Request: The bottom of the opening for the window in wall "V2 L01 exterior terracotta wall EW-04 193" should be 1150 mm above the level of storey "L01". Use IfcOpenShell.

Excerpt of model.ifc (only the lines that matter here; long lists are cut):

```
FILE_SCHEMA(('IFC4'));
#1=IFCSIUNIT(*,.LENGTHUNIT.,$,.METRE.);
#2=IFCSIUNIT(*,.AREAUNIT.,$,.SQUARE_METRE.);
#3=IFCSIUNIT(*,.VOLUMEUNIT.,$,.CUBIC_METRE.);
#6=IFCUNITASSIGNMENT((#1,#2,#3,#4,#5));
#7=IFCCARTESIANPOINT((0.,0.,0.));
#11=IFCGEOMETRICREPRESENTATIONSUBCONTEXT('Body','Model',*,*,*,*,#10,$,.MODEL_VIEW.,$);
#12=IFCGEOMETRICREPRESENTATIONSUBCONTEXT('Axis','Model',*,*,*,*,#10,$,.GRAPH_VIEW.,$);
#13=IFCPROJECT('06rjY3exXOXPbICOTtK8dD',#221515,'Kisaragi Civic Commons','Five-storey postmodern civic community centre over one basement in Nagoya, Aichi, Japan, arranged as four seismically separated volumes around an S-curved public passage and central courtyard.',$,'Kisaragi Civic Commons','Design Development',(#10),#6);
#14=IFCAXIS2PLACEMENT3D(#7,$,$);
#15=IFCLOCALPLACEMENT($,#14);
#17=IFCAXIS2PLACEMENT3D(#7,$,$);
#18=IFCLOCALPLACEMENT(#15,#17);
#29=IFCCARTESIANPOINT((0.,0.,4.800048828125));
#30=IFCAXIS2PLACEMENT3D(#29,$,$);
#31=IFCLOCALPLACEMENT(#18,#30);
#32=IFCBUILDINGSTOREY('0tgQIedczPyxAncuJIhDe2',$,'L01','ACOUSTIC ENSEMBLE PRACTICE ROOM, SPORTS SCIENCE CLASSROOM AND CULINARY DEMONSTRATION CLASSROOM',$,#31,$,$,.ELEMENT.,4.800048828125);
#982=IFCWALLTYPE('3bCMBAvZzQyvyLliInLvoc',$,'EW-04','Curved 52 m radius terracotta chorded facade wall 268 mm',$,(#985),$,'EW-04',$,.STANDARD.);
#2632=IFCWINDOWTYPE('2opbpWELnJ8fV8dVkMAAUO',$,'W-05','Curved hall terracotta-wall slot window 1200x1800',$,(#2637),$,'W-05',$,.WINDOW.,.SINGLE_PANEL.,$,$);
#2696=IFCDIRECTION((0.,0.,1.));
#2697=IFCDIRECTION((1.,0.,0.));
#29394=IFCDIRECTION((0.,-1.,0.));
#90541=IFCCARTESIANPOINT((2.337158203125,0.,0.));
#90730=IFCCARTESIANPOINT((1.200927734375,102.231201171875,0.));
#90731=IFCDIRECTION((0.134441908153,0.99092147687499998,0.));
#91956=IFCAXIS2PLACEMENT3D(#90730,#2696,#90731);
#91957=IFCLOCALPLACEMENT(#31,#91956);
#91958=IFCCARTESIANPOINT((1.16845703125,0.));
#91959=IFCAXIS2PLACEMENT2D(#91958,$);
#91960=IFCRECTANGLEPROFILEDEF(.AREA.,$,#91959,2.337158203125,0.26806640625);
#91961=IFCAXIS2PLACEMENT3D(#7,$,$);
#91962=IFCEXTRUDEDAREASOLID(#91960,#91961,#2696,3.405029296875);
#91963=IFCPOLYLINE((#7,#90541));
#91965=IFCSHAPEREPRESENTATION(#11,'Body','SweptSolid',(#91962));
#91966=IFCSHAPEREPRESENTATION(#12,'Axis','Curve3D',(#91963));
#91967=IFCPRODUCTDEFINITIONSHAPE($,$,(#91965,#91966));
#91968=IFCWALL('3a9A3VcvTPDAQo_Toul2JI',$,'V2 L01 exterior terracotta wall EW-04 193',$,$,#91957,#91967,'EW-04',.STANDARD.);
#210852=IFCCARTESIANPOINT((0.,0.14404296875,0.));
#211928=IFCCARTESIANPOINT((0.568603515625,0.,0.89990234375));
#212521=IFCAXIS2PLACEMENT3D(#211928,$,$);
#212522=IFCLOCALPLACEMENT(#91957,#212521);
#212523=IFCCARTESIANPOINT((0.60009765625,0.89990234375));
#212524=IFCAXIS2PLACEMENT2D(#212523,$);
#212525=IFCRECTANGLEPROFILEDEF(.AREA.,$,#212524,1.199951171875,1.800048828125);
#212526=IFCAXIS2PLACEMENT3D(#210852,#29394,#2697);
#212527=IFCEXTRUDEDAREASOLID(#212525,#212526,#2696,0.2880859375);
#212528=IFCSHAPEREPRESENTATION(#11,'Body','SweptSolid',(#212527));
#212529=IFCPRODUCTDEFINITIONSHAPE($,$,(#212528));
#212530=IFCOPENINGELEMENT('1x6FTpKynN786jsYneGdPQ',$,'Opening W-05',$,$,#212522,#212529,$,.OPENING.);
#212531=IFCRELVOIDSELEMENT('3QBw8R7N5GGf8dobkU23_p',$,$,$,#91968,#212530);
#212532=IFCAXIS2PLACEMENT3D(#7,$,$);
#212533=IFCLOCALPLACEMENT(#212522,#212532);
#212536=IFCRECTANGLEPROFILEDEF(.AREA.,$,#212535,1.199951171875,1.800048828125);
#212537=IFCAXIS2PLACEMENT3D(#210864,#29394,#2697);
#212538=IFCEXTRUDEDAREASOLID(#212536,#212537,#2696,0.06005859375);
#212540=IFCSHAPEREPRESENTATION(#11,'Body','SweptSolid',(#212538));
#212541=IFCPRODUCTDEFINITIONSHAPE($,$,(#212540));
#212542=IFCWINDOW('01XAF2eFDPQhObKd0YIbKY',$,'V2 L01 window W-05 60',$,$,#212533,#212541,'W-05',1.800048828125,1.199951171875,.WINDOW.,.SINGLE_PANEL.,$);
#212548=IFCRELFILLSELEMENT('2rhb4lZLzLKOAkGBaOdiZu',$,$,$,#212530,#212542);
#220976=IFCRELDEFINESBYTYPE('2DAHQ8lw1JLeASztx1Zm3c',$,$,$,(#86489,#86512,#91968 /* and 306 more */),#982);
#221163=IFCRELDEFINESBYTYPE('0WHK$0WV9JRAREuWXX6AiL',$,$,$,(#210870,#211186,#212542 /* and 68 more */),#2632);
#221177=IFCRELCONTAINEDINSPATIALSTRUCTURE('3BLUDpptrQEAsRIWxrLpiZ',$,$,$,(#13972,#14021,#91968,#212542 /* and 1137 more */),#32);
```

```python
import numpy as np
import ifcopenshell
import ifcopenshell.api.geometry
import ifcopenshell.geom
import ifcopenshell.util.element
import ifcopenshell.util.placement
import ifcopenshell.util.shape
import ifcopenshell.util.unit

model = ifcopenshell.open("model.ifc")
unit_scale = ifcopenshell.util.unit.calculate_unit_scale(model)

window = model.by_id(212542)
opening = window.FillsVoids[0].RelatingOpeningElement
storey = ifcopenshell.util.element.get_container(window, ifc_class="IfcBuildingStorey")
level = ifcopenshell.util.placement.get_local_placement(storey.ObjectPlacement)[2, 3]

# The opening's origin need not be at the sill, so measure its lowest point.
shape = ifcopenshell.geom.create_shape(ifcopenshell.geom.settings(), opening)
bottom = ifcopenshell.util.shape.get_shape_bottom_elevation(shape, shape.geometry) / unit_scale
dz = level + 1.15 / unit_scale - bottom

shift = np.array([0.0, 0.0, dz])
# The window is placed relative to its opening, so it follows when the opening moves.
matrix = ifcopenshell.util.placement.get_local_placement(opening.ObjectPlacement)
matrix[:3, 3] += shift
ifcopenshell.api.geometry.edit_object_placement(
    model, product=opening, matrix=matrix, is_si=False, should_transform_children=True
)

print(f"moved by {dz * unit_scale:+.3f} m")

model.write("model_updated.ifc")
```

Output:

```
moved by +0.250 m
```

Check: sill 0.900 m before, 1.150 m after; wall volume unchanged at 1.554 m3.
